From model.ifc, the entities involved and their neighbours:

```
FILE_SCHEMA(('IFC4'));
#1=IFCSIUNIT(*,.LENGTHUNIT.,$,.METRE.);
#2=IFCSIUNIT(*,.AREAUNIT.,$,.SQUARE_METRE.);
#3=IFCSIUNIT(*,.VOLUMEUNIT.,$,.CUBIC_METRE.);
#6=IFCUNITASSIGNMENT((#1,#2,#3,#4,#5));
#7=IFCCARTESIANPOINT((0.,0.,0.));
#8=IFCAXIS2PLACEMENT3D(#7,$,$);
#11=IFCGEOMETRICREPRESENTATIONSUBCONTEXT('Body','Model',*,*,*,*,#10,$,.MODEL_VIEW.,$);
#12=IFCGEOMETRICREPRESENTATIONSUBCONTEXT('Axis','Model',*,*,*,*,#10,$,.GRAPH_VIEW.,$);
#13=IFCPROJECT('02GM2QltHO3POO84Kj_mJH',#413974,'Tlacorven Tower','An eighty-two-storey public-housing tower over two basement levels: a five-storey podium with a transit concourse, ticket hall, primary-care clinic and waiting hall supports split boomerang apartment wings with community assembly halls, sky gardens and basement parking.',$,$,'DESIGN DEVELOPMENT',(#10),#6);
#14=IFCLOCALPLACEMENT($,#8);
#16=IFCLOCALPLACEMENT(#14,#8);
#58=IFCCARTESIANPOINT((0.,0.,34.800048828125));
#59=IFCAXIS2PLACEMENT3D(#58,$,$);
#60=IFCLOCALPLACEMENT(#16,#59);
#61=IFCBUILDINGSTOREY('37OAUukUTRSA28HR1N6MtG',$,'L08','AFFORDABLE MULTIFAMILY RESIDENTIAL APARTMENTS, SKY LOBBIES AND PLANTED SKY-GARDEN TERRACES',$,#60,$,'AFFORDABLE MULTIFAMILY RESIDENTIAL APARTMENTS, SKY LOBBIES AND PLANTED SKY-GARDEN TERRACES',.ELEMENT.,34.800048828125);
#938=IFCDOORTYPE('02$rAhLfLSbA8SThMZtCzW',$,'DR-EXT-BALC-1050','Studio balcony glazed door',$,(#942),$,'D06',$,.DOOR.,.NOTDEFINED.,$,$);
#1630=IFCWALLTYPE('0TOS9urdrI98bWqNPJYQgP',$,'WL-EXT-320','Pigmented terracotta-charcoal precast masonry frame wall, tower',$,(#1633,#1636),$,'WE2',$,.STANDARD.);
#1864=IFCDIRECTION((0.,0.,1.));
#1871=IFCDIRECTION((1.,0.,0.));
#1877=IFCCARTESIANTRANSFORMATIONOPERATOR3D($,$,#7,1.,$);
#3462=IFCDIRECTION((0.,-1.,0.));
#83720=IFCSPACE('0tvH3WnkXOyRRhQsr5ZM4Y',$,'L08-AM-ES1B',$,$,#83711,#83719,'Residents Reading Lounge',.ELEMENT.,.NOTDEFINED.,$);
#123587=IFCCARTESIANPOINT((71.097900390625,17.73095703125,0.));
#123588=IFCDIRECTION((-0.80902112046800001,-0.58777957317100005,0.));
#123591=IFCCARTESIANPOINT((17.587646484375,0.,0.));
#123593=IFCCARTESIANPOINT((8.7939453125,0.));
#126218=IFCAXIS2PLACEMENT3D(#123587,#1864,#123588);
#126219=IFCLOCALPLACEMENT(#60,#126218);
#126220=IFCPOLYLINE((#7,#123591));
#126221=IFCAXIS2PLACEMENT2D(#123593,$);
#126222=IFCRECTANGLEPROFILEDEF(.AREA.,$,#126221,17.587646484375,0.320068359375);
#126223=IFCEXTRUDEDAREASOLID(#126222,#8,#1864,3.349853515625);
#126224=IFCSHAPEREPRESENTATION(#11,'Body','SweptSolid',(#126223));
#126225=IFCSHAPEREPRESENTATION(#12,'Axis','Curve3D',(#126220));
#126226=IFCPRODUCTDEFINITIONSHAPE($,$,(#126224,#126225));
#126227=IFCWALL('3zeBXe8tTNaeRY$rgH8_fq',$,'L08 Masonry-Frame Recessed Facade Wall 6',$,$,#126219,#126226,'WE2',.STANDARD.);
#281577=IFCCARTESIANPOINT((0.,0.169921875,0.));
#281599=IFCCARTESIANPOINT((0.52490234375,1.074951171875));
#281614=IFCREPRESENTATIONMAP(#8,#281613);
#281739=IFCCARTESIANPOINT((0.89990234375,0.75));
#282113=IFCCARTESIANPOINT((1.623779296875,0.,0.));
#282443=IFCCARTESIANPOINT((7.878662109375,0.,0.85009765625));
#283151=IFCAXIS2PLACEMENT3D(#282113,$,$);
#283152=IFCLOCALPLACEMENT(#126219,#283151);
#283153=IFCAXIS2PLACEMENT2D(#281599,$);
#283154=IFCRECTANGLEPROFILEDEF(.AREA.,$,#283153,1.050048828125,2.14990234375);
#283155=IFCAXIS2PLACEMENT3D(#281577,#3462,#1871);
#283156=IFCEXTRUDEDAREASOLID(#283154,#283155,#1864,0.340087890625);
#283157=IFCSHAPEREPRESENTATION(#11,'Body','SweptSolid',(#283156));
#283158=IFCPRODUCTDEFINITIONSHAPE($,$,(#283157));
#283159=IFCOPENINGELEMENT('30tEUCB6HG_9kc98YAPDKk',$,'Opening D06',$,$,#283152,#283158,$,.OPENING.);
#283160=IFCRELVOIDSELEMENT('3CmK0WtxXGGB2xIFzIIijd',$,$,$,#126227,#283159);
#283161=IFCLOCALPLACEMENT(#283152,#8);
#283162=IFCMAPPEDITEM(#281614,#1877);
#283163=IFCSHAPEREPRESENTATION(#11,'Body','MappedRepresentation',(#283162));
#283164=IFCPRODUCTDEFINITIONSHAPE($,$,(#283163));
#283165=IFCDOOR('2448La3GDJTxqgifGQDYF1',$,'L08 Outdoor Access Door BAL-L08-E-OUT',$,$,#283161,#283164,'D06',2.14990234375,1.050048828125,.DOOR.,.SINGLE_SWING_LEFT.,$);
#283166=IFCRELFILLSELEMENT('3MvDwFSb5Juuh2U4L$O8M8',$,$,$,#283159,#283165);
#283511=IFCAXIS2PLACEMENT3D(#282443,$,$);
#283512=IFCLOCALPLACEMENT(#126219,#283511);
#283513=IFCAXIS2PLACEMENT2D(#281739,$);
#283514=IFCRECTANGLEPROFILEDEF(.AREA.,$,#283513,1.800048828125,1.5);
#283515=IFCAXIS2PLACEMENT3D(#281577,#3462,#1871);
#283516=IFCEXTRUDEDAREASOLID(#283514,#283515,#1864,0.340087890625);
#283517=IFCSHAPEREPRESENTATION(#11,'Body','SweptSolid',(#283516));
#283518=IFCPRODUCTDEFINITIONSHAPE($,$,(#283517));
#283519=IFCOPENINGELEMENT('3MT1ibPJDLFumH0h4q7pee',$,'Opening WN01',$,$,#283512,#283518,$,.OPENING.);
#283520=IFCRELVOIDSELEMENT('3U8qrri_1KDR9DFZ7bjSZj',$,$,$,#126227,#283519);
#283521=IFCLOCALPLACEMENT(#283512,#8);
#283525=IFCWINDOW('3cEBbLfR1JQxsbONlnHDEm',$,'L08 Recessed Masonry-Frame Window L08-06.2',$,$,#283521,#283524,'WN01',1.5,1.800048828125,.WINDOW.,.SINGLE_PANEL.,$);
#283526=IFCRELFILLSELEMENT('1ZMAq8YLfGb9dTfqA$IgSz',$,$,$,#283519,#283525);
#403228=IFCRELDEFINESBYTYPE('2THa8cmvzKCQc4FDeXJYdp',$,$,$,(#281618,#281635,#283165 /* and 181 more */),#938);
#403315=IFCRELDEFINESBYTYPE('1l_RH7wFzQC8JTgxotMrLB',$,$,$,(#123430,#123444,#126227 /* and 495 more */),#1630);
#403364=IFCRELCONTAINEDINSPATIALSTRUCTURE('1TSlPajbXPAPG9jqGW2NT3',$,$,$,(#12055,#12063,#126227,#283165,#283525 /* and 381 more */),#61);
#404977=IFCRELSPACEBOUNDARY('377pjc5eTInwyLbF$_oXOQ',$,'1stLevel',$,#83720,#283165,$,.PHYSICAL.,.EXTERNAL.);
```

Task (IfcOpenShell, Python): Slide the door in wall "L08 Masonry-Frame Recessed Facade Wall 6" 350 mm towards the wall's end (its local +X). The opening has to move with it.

```python
import ifcopenshell
import ifcopenshell.api.geometry
import ifcopenshell.util.placement

model = ifcopenshell.open("model.ifc")

door = model.by_guid("2448La3GDJTxqgifGQDYF1")
opening = door.FillsVoids[0].RelatingOpeningElement
wall = opening.VoidsElements[0].RelatingBuildingElement

wall_matrix = ifcopenshell.util.placement.get_local_placement(wall.ObjectPlacement)
shift = wall_matrix[:3, 0] * 0.35
before = ifcopenshell.util.placement.get_local_placement(door.ObjectPlacement)[:3, 3].copy()

# The door is placed relative to its opening, so it follows when the opening moves.
matrix = ifcopenshell.util.placement.get_local_placement(opening.ObjectPlacement)
matrix[:3, 3] += shift
ifcopenshell.api.geometry.edit_object_placement(
    model, product=opening, matrix=matrix, is_si=False, should_transform_children=True
)

after = ifcopenshell.util.placement.get_local_placement(door.ObjectPlacement)[:3, 3]
print("door moved by", (after - before).round(3) + 0.0)

model.write("model_updated.ifc")
```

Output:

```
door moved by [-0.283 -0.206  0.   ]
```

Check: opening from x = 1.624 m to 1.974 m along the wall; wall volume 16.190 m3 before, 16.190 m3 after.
